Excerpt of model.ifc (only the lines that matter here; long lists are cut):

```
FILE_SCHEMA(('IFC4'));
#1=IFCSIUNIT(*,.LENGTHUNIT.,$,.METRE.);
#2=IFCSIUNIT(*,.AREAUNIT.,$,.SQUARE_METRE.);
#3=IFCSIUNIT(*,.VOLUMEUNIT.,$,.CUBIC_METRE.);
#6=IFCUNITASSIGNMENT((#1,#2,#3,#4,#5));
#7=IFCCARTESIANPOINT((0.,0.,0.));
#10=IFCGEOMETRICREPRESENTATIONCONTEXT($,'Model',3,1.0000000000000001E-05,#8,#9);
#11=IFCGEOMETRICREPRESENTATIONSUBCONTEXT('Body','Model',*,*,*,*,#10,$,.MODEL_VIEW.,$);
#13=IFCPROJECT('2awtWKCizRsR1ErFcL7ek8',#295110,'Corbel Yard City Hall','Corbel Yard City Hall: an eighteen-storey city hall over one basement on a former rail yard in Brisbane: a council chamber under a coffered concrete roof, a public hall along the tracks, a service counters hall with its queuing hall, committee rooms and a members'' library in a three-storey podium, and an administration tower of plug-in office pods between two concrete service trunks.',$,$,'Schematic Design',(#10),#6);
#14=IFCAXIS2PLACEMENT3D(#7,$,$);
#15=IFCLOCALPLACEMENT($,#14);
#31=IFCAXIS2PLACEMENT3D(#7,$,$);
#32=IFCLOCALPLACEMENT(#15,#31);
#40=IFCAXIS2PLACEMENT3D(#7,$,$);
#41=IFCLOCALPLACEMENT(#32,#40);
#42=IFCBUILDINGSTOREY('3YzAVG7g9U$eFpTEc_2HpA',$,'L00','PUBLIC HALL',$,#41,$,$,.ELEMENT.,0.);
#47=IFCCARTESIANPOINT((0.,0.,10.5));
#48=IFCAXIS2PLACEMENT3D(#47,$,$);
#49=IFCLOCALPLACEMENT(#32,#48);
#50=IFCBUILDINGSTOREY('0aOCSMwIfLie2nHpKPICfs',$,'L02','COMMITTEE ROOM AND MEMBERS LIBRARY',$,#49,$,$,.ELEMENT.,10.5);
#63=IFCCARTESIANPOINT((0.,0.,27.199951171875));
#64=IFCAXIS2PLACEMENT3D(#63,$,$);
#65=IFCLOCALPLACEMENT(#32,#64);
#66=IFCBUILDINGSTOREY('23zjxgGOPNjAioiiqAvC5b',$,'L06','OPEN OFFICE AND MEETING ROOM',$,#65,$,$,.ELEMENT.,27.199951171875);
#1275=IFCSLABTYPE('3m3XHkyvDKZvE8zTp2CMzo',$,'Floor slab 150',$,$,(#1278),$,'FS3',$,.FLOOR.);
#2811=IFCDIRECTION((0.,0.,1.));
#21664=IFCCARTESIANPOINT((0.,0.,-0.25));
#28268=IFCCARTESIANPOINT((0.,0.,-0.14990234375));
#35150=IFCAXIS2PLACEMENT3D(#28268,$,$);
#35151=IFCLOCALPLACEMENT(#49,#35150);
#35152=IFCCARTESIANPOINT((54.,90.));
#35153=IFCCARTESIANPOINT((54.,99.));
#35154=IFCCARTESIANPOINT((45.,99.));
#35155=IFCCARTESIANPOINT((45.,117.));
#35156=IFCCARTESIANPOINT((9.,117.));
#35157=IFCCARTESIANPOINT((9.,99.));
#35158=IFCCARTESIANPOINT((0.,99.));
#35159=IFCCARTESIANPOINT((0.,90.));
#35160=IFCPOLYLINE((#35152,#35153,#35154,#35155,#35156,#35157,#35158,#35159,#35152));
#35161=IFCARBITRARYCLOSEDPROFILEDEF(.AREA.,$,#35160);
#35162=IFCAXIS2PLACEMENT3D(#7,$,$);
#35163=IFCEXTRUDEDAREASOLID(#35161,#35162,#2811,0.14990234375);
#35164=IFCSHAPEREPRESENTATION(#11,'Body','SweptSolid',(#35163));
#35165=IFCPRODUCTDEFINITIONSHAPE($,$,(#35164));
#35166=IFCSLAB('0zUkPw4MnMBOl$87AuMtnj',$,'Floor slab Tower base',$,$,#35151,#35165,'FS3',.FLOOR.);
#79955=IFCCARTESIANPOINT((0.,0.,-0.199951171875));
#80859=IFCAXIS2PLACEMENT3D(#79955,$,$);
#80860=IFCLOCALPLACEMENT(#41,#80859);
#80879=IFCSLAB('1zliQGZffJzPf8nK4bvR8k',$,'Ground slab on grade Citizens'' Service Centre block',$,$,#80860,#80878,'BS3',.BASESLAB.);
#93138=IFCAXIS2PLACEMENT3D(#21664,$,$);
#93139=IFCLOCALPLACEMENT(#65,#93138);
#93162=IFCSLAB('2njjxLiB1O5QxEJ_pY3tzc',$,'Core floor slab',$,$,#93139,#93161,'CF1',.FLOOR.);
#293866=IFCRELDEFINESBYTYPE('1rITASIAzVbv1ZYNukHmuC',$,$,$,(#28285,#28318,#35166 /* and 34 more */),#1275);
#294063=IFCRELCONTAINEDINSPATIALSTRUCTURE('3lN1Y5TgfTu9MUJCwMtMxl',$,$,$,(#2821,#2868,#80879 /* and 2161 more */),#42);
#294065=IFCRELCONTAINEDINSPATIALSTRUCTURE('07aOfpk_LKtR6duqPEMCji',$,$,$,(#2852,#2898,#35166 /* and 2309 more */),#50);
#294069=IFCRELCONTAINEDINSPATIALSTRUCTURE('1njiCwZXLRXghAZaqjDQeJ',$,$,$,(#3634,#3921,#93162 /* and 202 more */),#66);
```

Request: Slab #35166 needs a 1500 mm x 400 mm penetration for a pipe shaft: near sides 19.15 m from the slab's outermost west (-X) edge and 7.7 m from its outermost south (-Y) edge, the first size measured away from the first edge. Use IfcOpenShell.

```python
import numpy as np
import ifcopenshell
import ifcopenshell.api.feature
import ifcopenshell.api.geometry
import ifcopenshell.api.root
import ifcopenshell.geom
import ifcopenshell.util.placement
import ifcopenshell.util.representation
import ifcopenshell.util.shape
import ifcopenshell.util.unit

model = ifcopenshell.open("model.ifc")
unit_scale = ifcopenshell.util.unit.calculate_unit_scale(model)
settings = ifcopenshell.geom.settings()


def volume(element):
    """Net volume in cubic metres, openings subtracted."""
    shape = ifcopenshell.geom.create_shape(settings, element)
    return ifcopenshell.util.shape.get_volume(shape.geometry)


slab = model.by_guid("0zUkPw4MnMBOl$87AuMtnj")
before = volume(slab)

# Extent in the slab's own axes, in metres. The edges named are its -X and -Y sides.
slab_shape = ifcopenshell.geom.create_shape(settings, slab)
vertices = ifcopenshell.util.shape.get_vertices(slab_shape.geometry)
x_min, y_min, bottom = vertices.min(axis=0)
top = vertices[:, 2].max()

opening = ifcopenshell.api.root.create_entity(model, ifc_class="IfcOpeningElement", name="Pipe shaft opening", predefined_type="OPENING")
context = ifcopenshell.util.representation.get_context(model, "Model", "Body", "MODEL_VIEW")
width, depth = 1.5, 0.4
outline = [(0.0, 0.0), (width, 0.0), (width, depth), (0.0, depth), (0.0, 0.0)]
# Overshoot both faces by 50 mm so the cut is clean.
shape = ifcopenshell.api.geometry.add_slab_representation(
    model, context=context, depth=top - bottom + 0.1, polyline=outline
)
ifcopenshell.api.geometry.assign_representation(model, product=opening, representation=shape)

matrix = ifcopenshell.util.placement.get_local_placement(slab.ObjectPlacement)
matrix[:, 3] = matrix @ np.append(np.array([x_min + 19.15, y_min + 7.7, bottom - 0.05]) / unit_scale, 1.0)
ifcopenshell.api.geometry.edit_object_placement(model, product=opening, matrix=matrix, is_si=False)
ifcopenshell.api.feature.add_feature(model, feature=opening, element=slab)

after = volume(slab)

print(f"slab volume {before:.3f} -> {after:.3f} m3")

model.write("model_rev.ifc")
```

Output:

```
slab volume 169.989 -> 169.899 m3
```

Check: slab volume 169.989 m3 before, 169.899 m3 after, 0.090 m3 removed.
